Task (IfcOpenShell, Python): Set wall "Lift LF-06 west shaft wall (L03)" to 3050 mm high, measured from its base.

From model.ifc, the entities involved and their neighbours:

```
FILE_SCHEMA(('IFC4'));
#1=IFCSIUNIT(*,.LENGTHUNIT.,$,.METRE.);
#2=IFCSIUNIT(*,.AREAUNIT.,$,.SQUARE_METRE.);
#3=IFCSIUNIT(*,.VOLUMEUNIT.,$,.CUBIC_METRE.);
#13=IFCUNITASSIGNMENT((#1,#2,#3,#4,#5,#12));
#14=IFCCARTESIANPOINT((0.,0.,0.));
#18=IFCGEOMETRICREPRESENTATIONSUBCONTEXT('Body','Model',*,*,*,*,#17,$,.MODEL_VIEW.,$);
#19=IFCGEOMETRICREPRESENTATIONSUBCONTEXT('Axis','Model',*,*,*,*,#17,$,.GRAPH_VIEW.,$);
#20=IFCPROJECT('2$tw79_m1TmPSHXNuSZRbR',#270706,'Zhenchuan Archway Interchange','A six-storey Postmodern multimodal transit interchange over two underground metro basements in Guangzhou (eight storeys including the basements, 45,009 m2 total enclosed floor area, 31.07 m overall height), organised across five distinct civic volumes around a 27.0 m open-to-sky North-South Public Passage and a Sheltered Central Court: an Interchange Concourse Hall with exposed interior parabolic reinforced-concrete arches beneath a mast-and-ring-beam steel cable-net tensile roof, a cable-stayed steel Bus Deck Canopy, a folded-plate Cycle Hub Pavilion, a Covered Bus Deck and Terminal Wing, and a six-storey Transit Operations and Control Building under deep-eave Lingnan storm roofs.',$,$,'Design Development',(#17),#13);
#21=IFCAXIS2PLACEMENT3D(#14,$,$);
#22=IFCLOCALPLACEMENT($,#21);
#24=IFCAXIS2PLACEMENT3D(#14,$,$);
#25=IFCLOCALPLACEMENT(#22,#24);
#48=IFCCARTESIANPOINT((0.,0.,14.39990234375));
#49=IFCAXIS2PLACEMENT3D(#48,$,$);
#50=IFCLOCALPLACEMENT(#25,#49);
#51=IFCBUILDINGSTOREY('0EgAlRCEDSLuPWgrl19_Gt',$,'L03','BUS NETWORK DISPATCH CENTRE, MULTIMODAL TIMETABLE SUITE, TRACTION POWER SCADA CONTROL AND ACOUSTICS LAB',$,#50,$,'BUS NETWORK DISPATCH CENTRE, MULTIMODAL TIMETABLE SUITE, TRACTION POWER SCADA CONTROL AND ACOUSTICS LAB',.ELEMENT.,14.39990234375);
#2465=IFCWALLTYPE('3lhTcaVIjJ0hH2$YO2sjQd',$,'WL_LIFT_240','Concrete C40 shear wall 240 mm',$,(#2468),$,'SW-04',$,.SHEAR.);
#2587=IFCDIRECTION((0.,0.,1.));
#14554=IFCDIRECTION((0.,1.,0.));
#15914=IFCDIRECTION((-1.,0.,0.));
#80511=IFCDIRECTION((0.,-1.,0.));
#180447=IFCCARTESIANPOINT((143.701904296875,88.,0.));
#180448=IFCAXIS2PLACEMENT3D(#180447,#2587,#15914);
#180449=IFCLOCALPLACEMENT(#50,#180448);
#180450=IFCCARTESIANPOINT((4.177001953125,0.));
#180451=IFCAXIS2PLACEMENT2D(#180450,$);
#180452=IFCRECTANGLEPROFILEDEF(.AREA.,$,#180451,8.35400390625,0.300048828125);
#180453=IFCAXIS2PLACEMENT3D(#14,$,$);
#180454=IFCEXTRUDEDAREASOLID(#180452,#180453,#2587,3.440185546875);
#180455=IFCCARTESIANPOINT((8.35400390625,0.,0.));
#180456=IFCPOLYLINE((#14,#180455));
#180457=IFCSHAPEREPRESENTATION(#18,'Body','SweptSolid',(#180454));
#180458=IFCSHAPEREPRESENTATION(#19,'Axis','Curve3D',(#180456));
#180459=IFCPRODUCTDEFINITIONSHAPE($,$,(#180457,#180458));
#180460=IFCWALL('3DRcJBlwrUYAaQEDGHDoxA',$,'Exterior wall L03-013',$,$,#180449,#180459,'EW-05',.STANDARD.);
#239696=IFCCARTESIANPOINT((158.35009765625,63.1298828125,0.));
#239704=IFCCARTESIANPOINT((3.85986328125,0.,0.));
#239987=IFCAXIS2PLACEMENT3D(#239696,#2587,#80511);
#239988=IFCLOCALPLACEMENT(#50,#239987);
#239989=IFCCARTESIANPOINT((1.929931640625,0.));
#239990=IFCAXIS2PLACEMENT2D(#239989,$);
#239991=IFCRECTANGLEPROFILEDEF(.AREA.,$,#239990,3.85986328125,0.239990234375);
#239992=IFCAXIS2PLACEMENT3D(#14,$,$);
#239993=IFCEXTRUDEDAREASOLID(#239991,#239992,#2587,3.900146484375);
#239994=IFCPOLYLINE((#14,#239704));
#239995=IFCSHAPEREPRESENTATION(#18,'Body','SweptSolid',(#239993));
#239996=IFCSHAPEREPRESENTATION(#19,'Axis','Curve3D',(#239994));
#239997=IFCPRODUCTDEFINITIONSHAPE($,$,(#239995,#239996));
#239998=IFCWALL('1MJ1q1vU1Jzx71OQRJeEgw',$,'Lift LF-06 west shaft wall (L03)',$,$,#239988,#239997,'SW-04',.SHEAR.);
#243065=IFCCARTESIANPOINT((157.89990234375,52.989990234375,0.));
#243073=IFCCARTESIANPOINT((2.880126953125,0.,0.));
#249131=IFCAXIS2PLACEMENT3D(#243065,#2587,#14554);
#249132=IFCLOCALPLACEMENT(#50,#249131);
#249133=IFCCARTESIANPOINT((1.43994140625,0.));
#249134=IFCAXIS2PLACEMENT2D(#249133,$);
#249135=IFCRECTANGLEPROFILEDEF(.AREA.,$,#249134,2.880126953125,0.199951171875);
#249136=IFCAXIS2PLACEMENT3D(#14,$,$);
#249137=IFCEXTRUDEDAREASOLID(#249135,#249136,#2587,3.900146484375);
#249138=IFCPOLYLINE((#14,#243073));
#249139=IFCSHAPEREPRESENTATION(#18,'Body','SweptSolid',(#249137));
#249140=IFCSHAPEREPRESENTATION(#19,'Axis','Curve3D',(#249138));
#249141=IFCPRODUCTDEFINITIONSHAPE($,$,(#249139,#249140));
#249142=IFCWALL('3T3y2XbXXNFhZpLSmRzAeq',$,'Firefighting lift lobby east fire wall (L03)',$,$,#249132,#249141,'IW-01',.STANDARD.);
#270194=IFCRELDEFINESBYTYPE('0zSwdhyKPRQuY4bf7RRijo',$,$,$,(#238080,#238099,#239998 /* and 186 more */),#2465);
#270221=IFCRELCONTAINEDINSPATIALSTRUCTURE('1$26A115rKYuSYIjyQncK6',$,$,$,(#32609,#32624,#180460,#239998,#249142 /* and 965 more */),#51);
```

```python
import ifcopenshell
import ifcopenshell.geom
import ifcopenshell.util.representation
import ifcopenshell.util.shape

model = ifcopenshell.open("model.ifc")
settings = ifcopenshell.geom.settings()


def volume(element):
    """Net volume in cubic metres, openings subtracted."""
    shape = ifcopenshell.geom.create_shape(settings, element)
    return ifcopenshell.util.shape.get_volume(shape.geometry)


wall = model.by_guid("1MJ1q1vU1Jzx71OQRJeEgw")
before = volume(wall)

body = ifcopenshell.util.representation.get_representation(wall, "Model", "Body")
solid = body.Items[0]
old_height = solid.Depth
solid.Depth = 3.05
after = volume(wall)

print(f"height {old_height:g} -> {solid.Depth:g}, volume {before:.3f} -> {after:.3f} m3")

model.write("model_updated.ifc")
```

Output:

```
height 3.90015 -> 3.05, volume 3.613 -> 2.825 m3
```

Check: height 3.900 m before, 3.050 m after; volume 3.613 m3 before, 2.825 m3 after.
